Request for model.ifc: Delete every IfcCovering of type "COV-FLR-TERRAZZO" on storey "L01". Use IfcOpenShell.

First a look at what the model holds.

```python
import ifcopenshell
import ifcopenshell.util.element

model = ifcopenshell.open("model.ifc")
print(model.schema)
storey = next(s for s in model.by_type("IfcBuildingStorey") if s.Name == "L01")
coverings = [e for e in ifcopenshell.util.element.get_decomposition(storey) if e.is_a("IfcCovering")]
seen = {}
for e in coverings:
    element_type = ifcopenshell.util.element.get_type(e)
    name = element_type.Name if element_type not in (None, e) else None
    seen[name] = seen.get(name, 0) + 1
for name, count in sorted(seen.items(), key=str):
    print(count, "x", name)
```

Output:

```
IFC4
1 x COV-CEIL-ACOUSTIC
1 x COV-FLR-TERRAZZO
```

```python
import ifcopenshell
import ifcopenshell.api.root
import ifcopenshell.util.element

model = ifcopenshell.open("model.ifc")

storey = next(s for s in model.by_type("IfcBuildingStorey") if s.Name == "L01")
coverings = [e for e in ifcopenshell.util.element.get_decomposition(storey) if e.is_a("IfcCovering")]
targets = [e for e in coverings if (t := ifcopenshell.util.element.get_type(e)) not in (None, e) and t.Name == "COV-FLR-TERRAZZO"]

for e in targets:
    ifcopenshell.api.root.remove_product(model, product=e)
print(len(targets), "removed")

model.write("model_updated.ifc")
```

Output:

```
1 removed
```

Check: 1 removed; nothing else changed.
